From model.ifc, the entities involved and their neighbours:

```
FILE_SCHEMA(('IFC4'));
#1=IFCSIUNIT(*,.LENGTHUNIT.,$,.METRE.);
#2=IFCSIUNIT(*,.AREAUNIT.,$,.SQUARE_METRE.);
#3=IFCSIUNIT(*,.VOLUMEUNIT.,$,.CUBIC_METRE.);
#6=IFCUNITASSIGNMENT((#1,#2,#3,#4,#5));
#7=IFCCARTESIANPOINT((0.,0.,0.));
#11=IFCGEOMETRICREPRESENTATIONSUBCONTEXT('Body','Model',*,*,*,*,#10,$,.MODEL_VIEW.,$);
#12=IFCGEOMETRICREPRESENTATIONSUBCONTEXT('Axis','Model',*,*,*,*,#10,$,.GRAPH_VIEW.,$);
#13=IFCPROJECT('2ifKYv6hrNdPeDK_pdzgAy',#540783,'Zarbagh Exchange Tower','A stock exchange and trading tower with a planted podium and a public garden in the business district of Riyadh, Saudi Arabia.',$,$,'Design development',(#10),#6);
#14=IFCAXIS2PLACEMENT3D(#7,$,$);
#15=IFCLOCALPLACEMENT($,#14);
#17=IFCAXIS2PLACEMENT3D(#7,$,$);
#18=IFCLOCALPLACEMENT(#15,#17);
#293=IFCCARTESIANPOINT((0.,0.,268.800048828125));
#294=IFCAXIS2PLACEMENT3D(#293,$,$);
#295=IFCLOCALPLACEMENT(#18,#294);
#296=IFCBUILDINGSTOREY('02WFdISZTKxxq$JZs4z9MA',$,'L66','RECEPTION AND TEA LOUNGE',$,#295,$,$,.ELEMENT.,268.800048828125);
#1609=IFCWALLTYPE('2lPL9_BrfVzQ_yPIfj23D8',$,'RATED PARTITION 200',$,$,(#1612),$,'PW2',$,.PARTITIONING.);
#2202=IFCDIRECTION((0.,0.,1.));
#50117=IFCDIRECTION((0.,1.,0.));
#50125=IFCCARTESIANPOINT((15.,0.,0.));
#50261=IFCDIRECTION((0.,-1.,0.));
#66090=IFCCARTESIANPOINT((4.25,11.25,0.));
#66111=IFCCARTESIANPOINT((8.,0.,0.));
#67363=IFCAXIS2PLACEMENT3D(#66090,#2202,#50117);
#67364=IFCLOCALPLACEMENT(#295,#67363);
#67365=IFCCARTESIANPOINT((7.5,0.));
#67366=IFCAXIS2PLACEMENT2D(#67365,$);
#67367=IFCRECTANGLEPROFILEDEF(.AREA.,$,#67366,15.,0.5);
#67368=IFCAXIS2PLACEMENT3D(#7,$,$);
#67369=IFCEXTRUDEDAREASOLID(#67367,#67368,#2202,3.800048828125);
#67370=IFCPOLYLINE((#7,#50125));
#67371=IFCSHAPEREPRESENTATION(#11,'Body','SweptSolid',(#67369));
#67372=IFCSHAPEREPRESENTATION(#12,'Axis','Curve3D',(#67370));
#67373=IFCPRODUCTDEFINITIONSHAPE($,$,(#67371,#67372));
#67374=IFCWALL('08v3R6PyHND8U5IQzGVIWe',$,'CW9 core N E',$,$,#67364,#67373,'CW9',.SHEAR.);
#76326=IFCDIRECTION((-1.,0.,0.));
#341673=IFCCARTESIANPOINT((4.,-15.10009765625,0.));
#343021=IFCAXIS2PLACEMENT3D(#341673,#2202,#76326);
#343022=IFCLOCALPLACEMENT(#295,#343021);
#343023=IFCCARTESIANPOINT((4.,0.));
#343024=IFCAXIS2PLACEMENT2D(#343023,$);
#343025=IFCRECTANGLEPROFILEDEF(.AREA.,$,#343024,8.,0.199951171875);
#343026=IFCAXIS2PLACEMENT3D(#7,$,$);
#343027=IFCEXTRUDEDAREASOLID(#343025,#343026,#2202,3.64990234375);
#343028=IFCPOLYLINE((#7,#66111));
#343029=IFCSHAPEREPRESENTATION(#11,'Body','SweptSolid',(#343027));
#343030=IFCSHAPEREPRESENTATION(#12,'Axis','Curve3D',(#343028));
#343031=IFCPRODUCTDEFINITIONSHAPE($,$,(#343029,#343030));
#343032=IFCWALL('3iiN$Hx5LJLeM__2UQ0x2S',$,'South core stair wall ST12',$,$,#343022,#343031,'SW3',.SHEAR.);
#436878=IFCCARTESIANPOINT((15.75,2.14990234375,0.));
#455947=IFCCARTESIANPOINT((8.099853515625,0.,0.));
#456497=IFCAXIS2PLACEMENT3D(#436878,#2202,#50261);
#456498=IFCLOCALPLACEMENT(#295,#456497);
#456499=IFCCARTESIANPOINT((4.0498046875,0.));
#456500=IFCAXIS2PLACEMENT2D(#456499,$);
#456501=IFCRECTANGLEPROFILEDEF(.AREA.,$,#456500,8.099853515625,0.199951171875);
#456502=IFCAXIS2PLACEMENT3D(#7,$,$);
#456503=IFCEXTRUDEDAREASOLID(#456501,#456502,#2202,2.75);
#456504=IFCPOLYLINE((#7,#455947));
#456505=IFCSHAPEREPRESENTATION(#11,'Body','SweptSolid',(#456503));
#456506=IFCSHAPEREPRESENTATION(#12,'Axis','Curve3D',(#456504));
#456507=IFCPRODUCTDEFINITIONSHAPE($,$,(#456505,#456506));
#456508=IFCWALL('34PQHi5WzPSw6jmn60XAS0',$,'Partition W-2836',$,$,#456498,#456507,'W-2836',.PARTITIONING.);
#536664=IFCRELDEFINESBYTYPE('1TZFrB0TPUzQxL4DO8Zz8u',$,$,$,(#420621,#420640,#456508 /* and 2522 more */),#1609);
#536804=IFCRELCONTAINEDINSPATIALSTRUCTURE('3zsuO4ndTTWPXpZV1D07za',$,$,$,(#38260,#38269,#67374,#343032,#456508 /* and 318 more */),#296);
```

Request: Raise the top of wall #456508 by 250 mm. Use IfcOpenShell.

```python
import ifcopenshell
import ifcopenshell.geom
import ifcopenshell.util.representation
import ifcopenshell.util.shape

model = ifcopenshell.open("model.ifc")
settings = ifcopenshell.geom.settings()


def volume(element):
    """Net volume in cubic metres, openings subtracted."""
    shape = ifcopenshell.geom.create_shape(settings, element)
    return ifcopenshell.util.shape.get_volume(shape.geometry)


wall = model.by_id(456508)
before = volume(wall)

body = ifcopenshell.util.representation.get_representation(wall, "Model", "Body")
solid = body.Items[0]
old_height = solid.Depth
solid.Depth += 0.25
after = volume(wall)

print(f"height {old_height:g} -> {solid.Depth:g}, volume {before:.3f} -> {after:.3f} m3")

model.write("model_v2.ifc")
```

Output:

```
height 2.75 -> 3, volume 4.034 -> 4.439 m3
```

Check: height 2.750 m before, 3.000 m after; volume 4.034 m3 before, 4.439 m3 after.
